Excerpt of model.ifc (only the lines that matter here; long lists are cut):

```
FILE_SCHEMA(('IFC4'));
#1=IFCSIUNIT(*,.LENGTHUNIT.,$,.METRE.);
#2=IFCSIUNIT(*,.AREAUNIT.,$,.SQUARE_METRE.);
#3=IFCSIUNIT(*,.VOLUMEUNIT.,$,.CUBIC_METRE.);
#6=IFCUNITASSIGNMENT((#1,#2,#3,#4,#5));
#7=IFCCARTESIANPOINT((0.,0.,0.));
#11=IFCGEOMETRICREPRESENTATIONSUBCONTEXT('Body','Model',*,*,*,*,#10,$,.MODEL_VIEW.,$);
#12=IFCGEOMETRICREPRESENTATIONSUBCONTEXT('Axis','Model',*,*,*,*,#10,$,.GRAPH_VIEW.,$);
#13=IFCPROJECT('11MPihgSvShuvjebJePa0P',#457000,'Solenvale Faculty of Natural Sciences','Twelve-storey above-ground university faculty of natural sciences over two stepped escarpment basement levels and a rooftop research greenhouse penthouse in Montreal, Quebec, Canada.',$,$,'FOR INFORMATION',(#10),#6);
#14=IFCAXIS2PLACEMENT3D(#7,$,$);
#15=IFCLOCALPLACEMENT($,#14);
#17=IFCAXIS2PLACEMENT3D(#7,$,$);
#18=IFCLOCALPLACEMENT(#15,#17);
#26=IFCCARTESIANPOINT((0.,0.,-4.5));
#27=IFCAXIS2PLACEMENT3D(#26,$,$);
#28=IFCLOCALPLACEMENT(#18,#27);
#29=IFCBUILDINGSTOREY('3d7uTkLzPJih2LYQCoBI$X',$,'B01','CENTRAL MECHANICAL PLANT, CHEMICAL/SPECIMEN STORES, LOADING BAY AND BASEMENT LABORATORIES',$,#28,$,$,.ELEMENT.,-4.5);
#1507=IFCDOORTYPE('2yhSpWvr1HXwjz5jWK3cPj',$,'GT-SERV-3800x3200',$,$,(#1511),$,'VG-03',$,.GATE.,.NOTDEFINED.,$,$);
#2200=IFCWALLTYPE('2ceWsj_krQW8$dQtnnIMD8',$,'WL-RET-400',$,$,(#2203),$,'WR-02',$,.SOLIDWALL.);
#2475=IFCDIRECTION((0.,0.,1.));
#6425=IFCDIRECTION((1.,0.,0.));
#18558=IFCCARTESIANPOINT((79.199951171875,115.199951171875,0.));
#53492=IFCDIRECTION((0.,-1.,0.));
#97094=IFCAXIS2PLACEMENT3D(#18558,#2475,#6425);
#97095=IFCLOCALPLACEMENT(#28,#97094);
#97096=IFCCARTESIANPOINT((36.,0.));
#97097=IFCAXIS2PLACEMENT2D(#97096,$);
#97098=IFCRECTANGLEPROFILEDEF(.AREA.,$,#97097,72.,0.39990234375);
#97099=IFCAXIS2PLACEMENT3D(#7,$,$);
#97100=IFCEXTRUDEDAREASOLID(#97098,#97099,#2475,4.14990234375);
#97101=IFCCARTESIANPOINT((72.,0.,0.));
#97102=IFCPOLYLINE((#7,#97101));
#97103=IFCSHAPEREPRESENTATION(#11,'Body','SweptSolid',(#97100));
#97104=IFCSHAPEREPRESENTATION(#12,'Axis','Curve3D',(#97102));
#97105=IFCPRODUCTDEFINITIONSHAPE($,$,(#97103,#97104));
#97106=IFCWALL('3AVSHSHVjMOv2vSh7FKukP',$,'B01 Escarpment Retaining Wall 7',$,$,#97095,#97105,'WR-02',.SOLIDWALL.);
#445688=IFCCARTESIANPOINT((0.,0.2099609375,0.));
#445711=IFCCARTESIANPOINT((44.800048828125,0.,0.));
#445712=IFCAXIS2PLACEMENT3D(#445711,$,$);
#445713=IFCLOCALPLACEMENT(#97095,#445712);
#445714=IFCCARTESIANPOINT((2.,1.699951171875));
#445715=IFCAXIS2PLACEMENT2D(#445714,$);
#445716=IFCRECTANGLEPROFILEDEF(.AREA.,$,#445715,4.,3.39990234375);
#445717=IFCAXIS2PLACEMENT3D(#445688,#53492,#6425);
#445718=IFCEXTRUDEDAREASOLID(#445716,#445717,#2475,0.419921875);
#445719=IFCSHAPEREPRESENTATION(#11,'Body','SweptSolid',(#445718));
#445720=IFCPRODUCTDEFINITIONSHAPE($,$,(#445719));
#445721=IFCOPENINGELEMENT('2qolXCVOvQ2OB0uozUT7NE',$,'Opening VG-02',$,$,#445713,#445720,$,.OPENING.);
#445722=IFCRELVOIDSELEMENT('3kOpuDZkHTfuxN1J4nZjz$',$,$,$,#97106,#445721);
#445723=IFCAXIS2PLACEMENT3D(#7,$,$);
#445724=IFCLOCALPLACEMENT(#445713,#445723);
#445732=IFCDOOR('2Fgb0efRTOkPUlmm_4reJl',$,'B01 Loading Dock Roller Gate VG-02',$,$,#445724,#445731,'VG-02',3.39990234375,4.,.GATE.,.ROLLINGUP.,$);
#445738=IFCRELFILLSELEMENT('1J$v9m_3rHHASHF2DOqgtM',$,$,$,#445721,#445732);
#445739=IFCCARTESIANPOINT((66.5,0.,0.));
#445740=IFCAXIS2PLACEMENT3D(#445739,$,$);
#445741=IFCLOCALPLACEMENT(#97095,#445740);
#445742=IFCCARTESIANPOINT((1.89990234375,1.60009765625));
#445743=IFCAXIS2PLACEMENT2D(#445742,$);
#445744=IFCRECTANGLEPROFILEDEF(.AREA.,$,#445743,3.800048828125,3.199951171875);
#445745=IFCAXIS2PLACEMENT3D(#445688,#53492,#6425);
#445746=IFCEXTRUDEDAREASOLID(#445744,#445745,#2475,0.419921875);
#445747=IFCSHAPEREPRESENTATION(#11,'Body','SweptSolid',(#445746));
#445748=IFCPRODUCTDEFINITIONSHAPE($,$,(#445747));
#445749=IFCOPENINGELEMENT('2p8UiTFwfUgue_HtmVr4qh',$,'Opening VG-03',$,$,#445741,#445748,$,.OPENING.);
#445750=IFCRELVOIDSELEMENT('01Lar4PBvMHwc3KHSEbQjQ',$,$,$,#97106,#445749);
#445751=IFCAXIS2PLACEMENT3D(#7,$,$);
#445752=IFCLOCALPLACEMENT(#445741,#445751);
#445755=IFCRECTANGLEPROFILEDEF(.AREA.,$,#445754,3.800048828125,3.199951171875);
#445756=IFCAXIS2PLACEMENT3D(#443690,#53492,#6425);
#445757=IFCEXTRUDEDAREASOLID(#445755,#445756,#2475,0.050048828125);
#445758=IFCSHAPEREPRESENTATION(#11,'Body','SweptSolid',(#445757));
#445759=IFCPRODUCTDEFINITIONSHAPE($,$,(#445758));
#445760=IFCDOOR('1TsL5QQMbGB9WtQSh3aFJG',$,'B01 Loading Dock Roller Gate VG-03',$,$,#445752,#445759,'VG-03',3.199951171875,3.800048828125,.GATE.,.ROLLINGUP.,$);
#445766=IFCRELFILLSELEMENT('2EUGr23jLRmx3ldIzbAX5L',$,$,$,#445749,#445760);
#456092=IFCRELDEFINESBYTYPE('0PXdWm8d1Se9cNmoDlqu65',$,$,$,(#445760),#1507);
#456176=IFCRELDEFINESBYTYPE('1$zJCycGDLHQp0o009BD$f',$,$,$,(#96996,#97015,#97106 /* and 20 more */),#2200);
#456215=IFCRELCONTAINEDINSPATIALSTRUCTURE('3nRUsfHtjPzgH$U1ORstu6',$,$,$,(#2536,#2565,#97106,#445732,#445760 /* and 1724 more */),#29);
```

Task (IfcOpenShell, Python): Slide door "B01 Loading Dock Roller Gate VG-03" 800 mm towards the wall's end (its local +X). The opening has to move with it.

```python
import ifcopenshell
import ifcopenshell.api.geometry
import ifcopenshell.util.placement

model = ifcopenshell.open("model.ifc")

door = model.by_guid("1TsL5QQMbGB9WtQSh3aFJG")
opening = door.FillsVoids[0].RelatingOpeningElement
wall = opening.VoidsElements[0].RelatingBuildingElement

wall_matrix = ifcopenshell.util.placement.get_local_placement(wall.ObjectPlacement)
shift = wall_matrix[:3, 0] * 0.8
before = ifcopenshell.util.placement.get_local_placement(door.ObjectPlacement)[:3, 3].copy()

# The door is placed relative to its opening, so it follows when the opening moves.
matrix = ifcopenshell.util.placement.get_local_placement(opening.ObjectPlacement)
matrix[:3, 3] += shift
ifcopenshell.api.geometry.edit_object_placement(
    model, product=opening, matrix=matrix, is_si=False, should_transform_children=True
)

after = ifcopenshell.util.placement.get_local_placement(door.ObjectPlacement)[:3, 3]
print("door moved by", (after - before).round(3) + 0.0)

model.write("model_v2.ifc")
```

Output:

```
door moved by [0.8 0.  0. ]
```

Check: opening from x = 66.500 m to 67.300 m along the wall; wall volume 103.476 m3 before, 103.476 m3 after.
